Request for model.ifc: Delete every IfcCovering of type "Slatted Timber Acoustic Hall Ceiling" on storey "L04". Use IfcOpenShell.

First a look at what the model holds.

```python
import ifcopenshell
import ifcopenshell.util.element

model = ifcopenshell.open("model.ifc")
print(model.schema)
storey = next(s for s in model.by_type("IfcBuildingStorey") if s.Name == "L04")
coverings = [e for e in ifcopenshell.util.element.get_decomposition(storey) if e.is_a("IfcCovering")]
seen = {}
for e in coverings:
    element_type = ifcopenshell.util.element.get_type(e)
    name = element_type.Name if element_type not in (None, e) else None
    seen[name] = seen.get(name, 0) + 1
for name, count in sorted(seen.items(), key=str):
    print(count, "x", name)
```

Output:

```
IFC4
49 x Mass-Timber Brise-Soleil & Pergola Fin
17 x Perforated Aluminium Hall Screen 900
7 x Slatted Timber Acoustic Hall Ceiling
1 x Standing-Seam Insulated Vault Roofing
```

```python
import ifcopenshell
import ifcopenshell.api.root
import ifcopenshell.util.element

model = ifcopenshell.open("model.ifc")

storey = next(s for s in model.by_type("IfcBuildingStorey") if s.Name == "L04")
coverings = [e for e in ifcopenshell.util.element.get_decomposition(storey) if e.is_a("IfcCovering")]
targets = [e for e in coverings if (t := ifcopenshell.util.element.get_type(e)) not in (None, e) and t.Name == "Slatted Timber Acoustic Hall Ceiling"]

for e in targets:
    ifcopenshell.api.root.remove_product(model, product=e)
print(len(targets), "removed")

model.write("model-out.ifc")
```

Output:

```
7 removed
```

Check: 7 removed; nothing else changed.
